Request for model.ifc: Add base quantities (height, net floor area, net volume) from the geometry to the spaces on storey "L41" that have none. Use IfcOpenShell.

First a look at what the model holds.

```python
import ifcopenshell
import ifcopenshell.util.element
import ifcopenshell.util.unit

model = ifcopenshell.open("model.ifc")
print(model.schema)
for unit_type in ("LENGTHUNIT", "AREAUNIT", "VOLUMEUNIT"):
    print(unit_type, ifcopenshell.util.unit.calculate_unit_scale(model, unit_type))
storey = next(s for s in model.by_type("IfcBuildingStorey") if s.Name == "L41")
spaces = [e for e in ifcopenshell.util.element.get_decomposition(storey) if e.is_a("IfcSpace")]
for e in sorted(spaces, key=lambda e: e.id()):
    print(e.id(), e.is_a(), e.Name, list(ifcopenshell.util.element.get_psets(e, qtos_only=True)), sep=" | ")
```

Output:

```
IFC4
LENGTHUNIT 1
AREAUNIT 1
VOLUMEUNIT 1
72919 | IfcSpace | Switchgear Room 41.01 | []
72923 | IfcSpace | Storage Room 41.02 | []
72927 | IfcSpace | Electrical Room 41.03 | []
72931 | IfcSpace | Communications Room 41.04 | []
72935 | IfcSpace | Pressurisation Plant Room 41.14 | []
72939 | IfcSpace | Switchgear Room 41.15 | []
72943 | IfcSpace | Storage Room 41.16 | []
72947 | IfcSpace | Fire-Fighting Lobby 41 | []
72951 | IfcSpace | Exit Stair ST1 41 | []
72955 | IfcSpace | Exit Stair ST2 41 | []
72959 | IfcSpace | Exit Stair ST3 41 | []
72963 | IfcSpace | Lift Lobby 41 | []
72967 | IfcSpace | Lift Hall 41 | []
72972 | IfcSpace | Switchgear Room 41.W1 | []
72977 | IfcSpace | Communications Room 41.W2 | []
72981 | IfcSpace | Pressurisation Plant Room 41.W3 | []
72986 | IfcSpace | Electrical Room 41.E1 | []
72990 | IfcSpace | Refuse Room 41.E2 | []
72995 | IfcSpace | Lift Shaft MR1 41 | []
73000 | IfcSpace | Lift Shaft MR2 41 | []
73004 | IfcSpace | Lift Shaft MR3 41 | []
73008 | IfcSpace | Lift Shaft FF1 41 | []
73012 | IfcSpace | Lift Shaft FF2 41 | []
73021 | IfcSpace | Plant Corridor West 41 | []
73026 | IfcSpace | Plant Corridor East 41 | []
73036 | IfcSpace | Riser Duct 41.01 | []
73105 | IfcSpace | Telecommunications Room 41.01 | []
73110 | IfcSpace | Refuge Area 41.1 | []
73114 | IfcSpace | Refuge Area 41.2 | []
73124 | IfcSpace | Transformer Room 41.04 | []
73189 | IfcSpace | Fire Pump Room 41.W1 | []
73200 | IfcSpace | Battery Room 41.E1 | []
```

```python
import ifcopenshell
import ifcopenshell.api.pset
import ifcopenshell.geom
import ifcopenshell.util.element
import ifcopenshell.util.shape
import ifcopenshell.util.unit

model = ifcopenshell.open("model.ifc")
unit_scale = ifcopenshell.util.unit.calculate_unit_scale(model)
area_scale = ifcopenshell.util.unit.calculate_unit_scale(model, "AREAUNIT")
volume_scale = ifcopenshell.util.unit.calculate_unit_scale(model, "VOLUMEUNIT")
settings = ifcopenshell.geom.settings()

storey = next(s for s in model.by_type("IfcBuildingStorey") if s.Name == "L41")
spaces = [e for e in ifcopenshell.util.element.get_decomposition(storey) if e.is_a("IfcSpace")]

for e in sorted(spaces, key=lambda e: e.id()):
    if ifcopenshell.util.element.get_psets(e, qtos_only=True, should_inherit=False):
        continue
    # Geometry comes back in metres, in the element's own axes.
    shape = ifcopenshell.geom.create_shape(settings, e)
    values = {
        "Height": ifcopenshell.util.shape.get_z(shape.geometry) / unit_scale,
        "NetFloorArea": ifcopenshell.util.shape.get_footprint_area(shape.geometry) / area_scale,
        "NetVolume": ifcopenshell.util.shape.get_volume(shape.geometry) / volume_scale,
    }
    qto = ifcopenshell.api.pset.add_qto(model, product=e, name="Qto_SpaceBaseQuantities")
    ifcopenshell.api.pset.edit_qto(model, qto=qto, properties=values)
    print(e.id(), {k: round(v, 3) for k, v in values.items()})

model.write("model_edited.ifc")
```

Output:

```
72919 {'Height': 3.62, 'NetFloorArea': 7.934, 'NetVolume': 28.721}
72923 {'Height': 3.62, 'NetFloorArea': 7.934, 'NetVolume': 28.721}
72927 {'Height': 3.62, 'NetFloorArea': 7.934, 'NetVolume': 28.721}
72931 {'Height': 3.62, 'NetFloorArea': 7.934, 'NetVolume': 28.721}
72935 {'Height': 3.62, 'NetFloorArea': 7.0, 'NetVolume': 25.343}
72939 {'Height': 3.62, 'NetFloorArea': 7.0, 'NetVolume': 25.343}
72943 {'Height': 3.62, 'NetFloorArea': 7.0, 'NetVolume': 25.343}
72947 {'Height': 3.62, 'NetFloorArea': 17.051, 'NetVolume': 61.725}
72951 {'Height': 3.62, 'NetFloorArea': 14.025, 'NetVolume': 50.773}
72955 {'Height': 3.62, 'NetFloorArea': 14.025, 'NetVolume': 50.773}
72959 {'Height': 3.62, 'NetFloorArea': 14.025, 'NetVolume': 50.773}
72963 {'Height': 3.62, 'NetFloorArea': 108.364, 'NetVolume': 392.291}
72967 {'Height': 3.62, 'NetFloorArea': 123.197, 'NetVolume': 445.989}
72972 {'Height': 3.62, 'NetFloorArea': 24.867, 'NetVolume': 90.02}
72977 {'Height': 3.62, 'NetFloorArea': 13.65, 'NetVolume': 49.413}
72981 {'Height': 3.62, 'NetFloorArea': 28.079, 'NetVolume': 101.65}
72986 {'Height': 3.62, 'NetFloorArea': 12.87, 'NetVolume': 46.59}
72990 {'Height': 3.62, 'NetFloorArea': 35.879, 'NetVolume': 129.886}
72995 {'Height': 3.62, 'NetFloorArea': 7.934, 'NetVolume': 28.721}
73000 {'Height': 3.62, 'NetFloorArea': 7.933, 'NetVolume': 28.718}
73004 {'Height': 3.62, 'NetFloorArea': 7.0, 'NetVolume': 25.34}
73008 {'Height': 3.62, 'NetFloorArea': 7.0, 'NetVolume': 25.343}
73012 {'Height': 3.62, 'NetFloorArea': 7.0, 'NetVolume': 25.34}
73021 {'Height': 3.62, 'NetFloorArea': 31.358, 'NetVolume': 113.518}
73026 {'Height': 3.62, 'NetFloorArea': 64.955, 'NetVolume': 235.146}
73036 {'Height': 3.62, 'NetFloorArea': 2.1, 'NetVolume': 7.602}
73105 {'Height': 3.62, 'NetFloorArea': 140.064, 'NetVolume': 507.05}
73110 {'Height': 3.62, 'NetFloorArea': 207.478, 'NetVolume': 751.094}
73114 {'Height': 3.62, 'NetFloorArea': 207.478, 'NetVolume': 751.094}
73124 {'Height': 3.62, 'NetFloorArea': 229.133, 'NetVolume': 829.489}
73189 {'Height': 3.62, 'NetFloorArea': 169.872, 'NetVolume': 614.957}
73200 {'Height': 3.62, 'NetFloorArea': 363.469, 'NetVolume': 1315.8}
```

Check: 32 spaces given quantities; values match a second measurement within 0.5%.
